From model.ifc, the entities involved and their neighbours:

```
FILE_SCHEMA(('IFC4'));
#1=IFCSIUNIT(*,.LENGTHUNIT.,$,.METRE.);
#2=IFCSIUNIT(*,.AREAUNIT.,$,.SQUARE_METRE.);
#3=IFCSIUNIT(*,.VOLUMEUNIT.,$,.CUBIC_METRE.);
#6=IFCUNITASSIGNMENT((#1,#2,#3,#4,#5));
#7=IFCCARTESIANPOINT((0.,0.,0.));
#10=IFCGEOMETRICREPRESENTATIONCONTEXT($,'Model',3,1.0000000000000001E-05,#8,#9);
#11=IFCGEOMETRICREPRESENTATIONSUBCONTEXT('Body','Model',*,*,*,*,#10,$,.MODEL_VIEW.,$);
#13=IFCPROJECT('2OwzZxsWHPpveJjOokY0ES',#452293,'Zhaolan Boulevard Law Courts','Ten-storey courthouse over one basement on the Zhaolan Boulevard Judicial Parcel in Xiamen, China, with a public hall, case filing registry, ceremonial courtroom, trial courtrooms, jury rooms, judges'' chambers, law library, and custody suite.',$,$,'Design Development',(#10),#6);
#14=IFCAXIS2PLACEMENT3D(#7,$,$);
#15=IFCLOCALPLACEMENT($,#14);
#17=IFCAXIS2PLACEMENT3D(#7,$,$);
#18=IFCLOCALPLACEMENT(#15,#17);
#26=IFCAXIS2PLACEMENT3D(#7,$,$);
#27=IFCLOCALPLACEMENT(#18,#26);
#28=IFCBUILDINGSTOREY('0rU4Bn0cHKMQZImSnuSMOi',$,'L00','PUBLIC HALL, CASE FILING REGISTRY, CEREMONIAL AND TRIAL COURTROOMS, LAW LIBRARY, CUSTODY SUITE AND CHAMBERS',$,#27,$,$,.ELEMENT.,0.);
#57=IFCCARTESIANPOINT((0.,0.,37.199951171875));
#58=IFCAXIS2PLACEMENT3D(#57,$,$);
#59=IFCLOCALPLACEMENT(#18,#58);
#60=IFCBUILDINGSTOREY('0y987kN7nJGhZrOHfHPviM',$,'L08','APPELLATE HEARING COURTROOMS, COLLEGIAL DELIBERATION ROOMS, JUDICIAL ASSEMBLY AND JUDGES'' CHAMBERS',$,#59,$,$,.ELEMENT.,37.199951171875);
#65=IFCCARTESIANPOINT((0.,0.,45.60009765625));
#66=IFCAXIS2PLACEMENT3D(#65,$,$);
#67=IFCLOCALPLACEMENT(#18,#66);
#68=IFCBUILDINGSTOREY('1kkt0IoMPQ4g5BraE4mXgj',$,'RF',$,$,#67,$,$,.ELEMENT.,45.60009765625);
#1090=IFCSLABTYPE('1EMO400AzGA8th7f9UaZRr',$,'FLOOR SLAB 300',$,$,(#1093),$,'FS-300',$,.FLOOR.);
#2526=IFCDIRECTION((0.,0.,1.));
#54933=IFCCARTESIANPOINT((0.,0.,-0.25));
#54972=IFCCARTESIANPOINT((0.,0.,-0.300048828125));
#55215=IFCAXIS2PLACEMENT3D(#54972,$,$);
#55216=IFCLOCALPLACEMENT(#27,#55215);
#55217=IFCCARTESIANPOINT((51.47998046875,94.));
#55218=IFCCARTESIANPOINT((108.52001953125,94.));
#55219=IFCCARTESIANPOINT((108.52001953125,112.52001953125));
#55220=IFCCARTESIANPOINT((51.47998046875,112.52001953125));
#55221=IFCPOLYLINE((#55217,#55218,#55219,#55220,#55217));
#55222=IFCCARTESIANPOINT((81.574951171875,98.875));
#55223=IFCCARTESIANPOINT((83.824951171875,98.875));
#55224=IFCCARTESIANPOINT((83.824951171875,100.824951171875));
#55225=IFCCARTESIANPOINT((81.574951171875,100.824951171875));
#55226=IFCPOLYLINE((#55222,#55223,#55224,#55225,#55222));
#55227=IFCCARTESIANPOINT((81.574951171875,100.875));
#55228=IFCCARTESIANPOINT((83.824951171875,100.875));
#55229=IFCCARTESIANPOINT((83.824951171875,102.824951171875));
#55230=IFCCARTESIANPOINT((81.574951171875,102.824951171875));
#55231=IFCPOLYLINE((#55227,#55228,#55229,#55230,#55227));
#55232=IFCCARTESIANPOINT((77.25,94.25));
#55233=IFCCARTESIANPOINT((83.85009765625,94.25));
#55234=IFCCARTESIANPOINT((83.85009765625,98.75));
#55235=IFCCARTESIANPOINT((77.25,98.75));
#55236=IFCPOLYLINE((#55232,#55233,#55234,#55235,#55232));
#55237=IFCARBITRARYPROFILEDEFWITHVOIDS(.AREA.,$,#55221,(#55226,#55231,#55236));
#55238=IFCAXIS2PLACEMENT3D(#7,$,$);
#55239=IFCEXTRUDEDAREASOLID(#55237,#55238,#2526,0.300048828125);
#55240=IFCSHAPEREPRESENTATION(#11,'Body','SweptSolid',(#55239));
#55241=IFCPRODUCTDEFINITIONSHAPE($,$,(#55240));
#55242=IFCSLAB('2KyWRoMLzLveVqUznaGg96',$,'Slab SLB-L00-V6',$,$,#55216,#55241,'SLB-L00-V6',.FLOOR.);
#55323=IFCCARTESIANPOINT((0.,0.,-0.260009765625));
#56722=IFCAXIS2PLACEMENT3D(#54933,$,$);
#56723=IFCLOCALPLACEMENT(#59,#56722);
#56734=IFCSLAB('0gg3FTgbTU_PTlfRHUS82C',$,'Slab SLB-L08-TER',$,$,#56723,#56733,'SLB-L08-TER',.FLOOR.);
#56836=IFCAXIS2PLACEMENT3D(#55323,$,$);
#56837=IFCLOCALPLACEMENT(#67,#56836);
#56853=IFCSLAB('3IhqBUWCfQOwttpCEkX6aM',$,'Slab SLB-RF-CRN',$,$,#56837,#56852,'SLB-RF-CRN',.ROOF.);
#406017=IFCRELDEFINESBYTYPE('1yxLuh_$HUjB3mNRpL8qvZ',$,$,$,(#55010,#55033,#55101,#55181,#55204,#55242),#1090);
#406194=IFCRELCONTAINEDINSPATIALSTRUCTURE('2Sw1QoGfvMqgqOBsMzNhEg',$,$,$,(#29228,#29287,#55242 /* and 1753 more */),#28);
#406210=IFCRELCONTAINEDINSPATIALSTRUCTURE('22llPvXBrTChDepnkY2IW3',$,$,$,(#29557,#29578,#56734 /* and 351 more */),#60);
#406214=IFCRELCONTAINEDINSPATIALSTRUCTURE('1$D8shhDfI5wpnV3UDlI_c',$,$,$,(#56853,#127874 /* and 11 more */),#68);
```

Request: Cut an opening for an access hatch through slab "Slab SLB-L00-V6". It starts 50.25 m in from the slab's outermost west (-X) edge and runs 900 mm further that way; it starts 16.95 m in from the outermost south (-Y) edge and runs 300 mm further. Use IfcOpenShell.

```python
import numpy as np
import ifcopenshell
import ifcopenshell.api.feature
import ifcopenshell.api.geometry
import ifcopenshell.api.root
import ifcopenshell.geom
import ifcopenshell.util.placement
import ifcopenshell.util.representation
import ifcopenshell.util.shape
import ifcopenshell.util.unit

model = ifcopenshell.open("model.ifc")
unit_scale = ifcopenshell.util.unit.calculate_unit_scale(model)
settings = ifcopenshell.geom.settings()


def volume(element):
    """Net volume in cubic metres, openings subtracted."""
    shape = ifcopenshell.geom.create_shape(settings, element)
    return ifcopenshell.util.shape.get_volume(shape.geometry)


slab = model.by_guid("2KyWRoMLzLveVqUznaGg96")
before = volume(slab)

# Extent in the slab's own axes, in metres. The edges named are its -X and -Y sides.
slab_shape = ifcopenshell.geom.create_shape(settings, slab)
vertices = ifcopenshell.util.shape.get_vertices(slab_shape.geometry)
x_min, y_min, bottom = vertices.min(axis=0)
top = vertices[:, 2].max()

opening = ifcopenshell.api.root.create_entity(model, ifc_class="IfcOpeningElement", name="Access hatch opening", predefined_type="OPENING")
context = ifcopenshell.util.representation.get_context(model, "Model", "Body", "MODEL_VIEW")
width, depth = 0.9, 0.3
outline = [(0.0, 0.0), (width, 0.0), (width, depth), (0.0, depth), (0.0, 0.0)]
# Overshoot both faces by 50 mm so the cut is clean.
shape = ifcopenshell.api.geometry.add_slab_representation(
    model, context=context, depth=top - bottom + 0.1, polyline=outline
)
ifcopenshell.api.geometry.assign_representation(model, product=opening, representation=shape)

matrix = ifcopenshell.util.placement.get_local_placement(slab.ObjectPlacement)
matrix[:, 3] = matrix @ np.append(np.array([x_min + 50.25, y_min + 16.95, bottom - 0.05]) / unit_scale, 1.0)
ifcopenshell.api.geometry.edit_object_placement(model, product=opening, matrix=matrix, is_si=False)
ifcopenshell.api.feature.add_feature(model, feature=opening, element=slab)

after = volume(slab)

print(f"slab volume {before:.3f} -> {after:.3f} m3")

model.write("model_v2.ifc")
```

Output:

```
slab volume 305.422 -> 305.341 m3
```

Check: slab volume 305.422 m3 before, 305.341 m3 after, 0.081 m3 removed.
